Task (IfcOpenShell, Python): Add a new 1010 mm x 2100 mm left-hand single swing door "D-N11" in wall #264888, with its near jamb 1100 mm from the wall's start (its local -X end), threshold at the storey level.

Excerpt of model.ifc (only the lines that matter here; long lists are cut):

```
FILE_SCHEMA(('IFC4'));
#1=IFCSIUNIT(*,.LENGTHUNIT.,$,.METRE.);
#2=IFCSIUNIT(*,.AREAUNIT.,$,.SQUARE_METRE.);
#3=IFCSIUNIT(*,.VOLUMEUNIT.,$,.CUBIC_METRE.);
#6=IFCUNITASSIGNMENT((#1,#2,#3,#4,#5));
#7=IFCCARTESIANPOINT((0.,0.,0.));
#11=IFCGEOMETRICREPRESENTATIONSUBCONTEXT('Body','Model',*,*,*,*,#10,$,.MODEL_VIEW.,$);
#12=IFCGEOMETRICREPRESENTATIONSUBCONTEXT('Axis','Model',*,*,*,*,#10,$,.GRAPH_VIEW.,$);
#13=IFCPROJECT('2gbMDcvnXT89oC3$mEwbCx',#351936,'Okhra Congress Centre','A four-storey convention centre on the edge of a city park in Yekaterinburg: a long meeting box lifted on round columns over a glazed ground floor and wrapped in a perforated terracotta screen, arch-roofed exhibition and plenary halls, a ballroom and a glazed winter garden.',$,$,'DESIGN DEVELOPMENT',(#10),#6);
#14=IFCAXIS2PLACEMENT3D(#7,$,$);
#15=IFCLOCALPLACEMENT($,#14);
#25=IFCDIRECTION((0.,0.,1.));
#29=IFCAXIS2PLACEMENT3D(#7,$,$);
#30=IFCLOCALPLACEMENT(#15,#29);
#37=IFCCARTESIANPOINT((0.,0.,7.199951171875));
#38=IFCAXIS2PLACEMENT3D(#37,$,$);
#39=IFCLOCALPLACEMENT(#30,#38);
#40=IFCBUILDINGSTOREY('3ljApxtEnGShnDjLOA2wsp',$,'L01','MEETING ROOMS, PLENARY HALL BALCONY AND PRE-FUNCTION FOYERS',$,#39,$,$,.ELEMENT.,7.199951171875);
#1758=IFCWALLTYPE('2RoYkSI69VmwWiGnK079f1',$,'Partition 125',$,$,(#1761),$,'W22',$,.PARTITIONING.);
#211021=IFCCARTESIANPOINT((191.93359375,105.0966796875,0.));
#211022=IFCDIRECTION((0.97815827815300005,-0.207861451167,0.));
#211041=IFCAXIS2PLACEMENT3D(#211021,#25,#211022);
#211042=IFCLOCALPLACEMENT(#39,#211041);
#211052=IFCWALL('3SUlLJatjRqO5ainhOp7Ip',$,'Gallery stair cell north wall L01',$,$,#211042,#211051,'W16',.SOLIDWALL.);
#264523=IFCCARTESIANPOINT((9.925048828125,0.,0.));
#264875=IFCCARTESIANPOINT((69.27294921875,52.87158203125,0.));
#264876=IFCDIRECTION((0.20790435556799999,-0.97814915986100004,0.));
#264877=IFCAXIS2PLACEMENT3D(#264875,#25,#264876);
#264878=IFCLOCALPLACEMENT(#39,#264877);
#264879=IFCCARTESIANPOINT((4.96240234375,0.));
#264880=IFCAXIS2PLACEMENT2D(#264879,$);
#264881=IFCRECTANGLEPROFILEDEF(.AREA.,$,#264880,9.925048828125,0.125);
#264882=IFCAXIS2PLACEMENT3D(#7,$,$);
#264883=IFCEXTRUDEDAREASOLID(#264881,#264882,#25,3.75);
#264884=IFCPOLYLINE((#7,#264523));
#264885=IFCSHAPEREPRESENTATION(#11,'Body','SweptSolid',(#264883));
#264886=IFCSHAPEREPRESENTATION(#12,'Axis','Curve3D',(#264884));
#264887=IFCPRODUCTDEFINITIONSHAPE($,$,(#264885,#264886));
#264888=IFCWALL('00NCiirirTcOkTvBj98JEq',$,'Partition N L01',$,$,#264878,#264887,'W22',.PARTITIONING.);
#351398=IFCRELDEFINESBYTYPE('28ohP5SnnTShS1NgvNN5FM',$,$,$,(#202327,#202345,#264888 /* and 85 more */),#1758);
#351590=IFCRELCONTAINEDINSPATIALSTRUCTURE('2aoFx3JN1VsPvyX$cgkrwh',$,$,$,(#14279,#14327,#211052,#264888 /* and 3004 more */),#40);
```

```python
import numpy as np
import ifcopenshell
import ifcopenshell.api.feature
import ifcopenshell.api.geometry
import ifcopenshell.api.root
import ifcopenshell.api.spatial
import ifcopenshell.geom
import ifcopenshell.util.element
import ifcopenshell.util.placement
import ifcopenshell.util.representation
import ifcopenshell.util.shape
import ifcopenshell.util.unit

model = ifcopenshell.open("model.ifc")
unit_scale = ifcopenshell.util.unit.calculate_unit_scale(model)
settings = ifcopenshell.geom.settings()


def volume(element):
    """Net volume in cubic metres, openings subtracted."""
    shape = ifcopenshell.geom.create_shape(settings, element)
    return ifcopenshell.util.shape.get_volume(shape.geometry)


wall = model.by_id(264888)
storey = ifcopenshell.util.element.get_container(wall, ifc_class="IfcBuildingStorey")
context = ifcopenshell.util.representation.get_context(model, "Model", "Body", "MODEL_VIEW")
before = volume(wall)

width, height, from_end, sill = 1.01, 2.1, 1.1, 0.0  # metres

# The wall runs along its own X axis, and the end named is its -X end.
wall_shape = ifcopenshell.geom.create_shape(settings, wall)
x, y, z = ifcopenshell.util.shape.get_vertices(wall_shape.geometry).T
start = x.min() + from_end
face, thickness = float(y.min()), float(y.max() - y.min())
wall_matrix = ifcopenshell.util.placement.get_local_placement(wall.ObjectPlacement)
level = ifcopenshell.util.placement.get_local_placement(storey.ObjectPlacement)[2, 3]


def in_wall(x, y):
    """Placement at x, y metres in the wall's axes, at sill height."""
    matrix = wall_matrix.copy()
    matrix[:, 3] = wall_matrix @ np.array([x / unit_scale, y / unit_scale, 0.0, 1.0])
    matrix[2, 3] = level + sill / unit_scale
    return matrix


# Opening: a box that overshoots both wall faces by 50 mm.
opening = ifcopenshell.api.root.create_entity(model, ifc_class="IfcOpeningElement", predefined_type="OPENING")
box = ifcopenshell.api.geometry.add_wall_representation(
    model, context=context, length=width, height=height, thickness=thickness + 0.1
)
ifcopenshell.api.geometry.assign_representation(model, product=opening, representation=box)
ifcopenshell.api.geometry.edit_object_placement(model, product=opening, matrix=in_wall(start, face - 0.05), is_si=False)
ifcopenshell.api.feature.add_feature(model, feature=opening, element=wall)

door = ifcopenshell.api.root.create_entity(model, ifc_class="IfcDoor", name="D-N11", predefined_type="DOOR")
door.OverallWidth, door.OverallHeight = width / unit_scale, height / unit_scale
door.OperationType = "SINGLE_SWING_LEFT"
body = ifcopenshell.api.geometry.add_door_representation(
    model,
    context=context,
    overall_width=door.OverallWidth,
    overall_height=door.OverallHeight,
    operation_type="SINGLE_SWING_LEFT",
    lining_properties={"LiningDepth": thickness / unit_scale, "ThresholdDepth": thickness / unit_scale},
)
ifcopenshell.api.geometry.assign_representation(model, product=door, representation=body)
ifcopenshell.api.spatial.assign_container(model, products=[door], relating_structure=storey)
ifcopenshell.api.feature.add_filling(model, opening=opening, element=door)

# The lining spans the wall, so the door starts at the wall face.
ifcopenshell.api.geometry.edit_object_placement(model, product=door, matrix=in_wall(start, face), is_si=False)

after = volume(wall)

print(f"wall volume {before:.3f} -> {after:.3f} m3")

model.write("model_v2.ifc")
```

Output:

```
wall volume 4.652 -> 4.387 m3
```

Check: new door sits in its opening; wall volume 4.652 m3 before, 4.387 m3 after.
